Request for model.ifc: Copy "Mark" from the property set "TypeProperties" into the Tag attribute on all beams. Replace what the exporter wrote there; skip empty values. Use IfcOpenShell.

First a look at what the model holds.

```python
import ifcopenshell
import ifcopenshell.util.element

model = ifcopenshell.open("model.ifc")
print(model.schema)
beams = model.by_type("IfcBeam")
print(len(beams), "beams")
for e in beams[:8]:
    source = ifcopenshell.util.element.get_pset(e, "TypeProperties", "Mark")
    target = e.Tag
    print(e.id(), repr(source), repr(target), sep=" | ")
```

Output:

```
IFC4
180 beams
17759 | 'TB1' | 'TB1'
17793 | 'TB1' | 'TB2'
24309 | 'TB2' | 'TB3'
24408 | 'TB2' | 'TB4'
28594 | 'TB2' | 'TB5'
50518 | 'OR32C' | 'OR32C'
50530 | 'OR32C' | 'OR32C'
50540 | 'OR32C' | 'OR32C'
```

```python
import ifcopenshell
import ifcopenshell.util.element

model = ifcopenshell.open("model.ifc")

count = 0
for e in model.by_type("IfcBeam"):
    value = ifcopenshell.util.element.get_pset(e, "TypeProperties", "Mark")
    current = e.Tag
    if not value or not value.strip() or current == value:
        continue
    e.Tag = value
    count += 1

print(count, "beams updated")

model.write("model_rev.ifc")
```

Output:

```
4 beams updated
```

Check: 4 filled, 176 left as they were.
